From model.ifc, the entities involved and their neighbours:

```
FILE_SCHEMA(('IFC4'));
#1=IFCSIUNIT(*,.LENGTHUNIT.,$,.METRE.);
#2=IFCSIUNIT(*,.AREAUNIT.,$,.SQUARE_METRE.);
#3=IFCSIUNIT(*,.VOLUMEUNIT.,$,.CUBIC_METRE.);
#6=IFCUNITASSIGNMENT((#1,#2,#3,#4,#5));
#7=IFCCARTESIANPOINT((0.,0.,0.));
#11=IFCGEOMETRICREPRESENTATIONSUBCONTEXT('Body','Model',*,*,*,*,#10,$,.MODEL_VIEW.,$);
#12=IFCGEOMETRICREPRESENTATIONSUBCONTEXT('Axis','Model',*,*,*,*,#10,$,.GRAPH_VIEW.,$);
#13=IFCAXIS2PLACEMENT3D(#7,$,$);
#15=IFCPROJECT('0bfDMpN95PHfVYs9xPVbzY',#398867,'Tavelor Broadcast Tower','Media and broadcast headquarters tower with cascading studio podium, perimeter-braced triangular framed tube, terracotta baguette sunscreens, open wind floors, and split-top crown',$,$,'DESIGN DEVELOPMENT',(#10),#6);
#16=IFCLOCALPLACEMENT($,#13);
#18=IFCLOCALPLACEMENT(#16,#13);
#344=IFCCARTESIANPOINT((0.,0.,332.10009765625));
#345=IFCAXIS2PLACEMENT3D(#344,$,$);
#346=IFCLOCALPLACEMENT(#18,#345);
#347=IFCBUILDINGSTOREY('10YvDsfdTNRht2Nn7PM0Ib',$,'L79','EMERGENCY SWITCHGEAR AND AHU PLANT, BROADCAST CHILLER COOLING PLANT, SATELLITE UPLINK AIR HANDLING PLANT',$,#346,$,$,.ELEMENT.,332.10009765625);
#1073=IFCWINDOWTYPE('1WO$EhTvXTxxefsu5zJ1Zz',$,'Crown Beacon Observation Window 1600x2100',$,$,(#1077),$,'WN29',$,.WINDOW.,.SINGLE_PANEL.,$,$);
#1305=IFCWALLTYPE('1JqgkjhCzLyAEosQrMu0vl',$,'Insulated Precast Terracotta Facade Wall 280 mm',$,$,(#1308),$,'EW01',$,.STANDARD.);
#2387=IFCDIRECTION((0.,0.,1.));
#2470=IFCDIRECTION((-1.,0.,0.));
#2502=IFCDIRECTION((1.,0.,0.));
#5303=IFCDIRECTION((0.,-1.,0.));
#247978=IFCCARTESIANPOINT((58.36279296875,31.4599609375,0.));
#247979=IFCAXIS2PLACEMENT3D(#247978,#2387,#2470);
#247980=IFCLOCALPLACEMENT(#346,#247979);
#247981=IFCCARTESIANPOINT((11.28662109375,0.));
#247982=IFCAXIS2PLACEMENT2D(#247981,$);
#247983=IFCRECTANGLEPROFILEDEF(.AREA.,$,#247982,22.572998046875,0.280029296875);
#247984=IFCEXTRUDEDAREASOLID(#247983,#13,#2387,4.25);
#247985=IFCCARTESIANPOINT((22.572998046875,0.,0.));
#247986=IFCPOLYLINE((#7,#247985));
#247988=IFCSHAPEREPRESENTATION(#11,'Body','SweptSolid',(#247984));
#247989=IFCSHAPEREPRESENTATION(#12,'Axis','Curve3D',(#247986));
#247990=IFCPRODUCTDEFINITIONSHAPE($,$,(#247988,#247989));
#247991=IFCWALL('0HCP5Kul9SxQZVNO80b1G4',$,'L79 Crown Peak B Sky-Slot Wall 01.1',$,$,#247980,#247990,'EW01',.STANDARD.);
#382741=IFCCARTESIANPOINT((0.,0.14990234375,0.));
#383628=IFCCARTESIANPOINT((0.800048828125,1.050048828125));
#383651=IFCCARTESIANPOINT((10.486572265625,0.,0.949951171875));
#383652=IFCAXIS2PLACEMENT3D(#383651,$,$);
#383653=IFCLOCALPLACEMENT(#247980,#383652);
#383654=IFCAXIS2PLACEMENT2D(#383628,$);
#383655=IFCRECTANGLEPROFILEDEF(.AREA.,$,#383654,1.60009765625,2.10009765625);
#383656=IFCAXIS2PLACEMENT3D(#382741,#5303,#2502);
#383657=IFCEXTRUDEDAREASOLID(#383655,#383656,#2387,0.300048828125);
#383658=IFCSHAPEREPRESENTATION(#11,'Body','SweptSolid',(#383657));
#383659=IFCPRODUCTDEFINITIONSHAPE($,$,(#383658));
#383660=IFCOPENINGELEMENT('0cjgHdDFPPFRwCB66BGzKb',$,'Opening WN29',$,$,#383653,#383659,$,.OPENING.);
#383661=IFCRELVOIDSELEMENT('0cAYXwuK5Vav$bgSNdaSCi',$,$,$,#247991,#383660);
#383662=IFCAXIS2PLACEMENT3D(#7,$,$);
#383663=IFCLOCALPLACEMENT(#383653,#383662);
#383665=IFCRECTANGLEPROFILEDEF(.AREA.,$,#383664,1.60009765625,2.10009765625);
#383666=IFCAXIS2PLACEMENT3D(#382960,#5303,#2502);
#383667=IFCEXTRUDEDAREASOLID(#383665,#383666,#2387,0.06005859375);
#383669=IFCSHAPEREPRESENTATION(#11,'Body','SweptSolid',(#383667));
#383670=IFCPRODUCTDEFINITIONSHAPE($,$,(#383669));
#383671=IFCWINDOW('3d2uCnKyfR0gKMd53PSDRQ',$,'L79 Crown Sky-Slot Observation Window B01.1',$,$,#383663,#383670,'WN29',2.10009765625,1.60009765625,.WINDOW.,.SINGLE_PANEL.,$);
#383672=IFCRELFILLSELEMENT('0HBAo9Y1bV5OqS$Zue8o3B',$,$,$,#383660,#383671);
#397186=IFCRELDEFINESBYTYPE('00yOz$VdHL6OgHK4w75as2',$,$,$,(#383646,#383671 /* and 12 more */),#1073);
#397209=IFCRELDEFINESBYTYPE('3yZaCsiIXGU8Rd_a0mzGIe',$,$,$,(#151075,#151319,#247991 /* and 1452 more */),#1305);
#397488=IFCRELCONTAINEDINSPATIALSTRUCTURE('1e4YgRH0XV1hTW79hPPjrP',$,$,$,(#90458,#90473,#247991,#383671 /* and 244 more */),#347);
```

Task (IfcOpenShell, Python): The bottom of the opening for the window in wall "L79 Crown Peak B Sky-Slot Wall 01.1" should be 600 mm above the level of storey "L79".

```python
import numpy as np
import ifcopenshell
import ifcopenshell.api.geometry
import ifcopenshell.geom
import ifcopenshell.util.element
import ifcopenshell.util.placement
import ifcopenshell.util.shape
import ifcopenshell.util.unit

model = ifcopenshell.open("model.ifc")
unit_scale = ifcopenshell.util.unit.calculate_unit_scale(model)

window = model.by_guid("3d2uCnKyfR0gKMd53PSDRQ")
opening = window.FillsVoids[0].RelatingOpeningElement
storey = ifcopenshell.util.element.get_container(window, ifc_class="IfcBuildingStorey")
level = ifcopenshell.util.placement.get_local_placement(storey.ObjectPlacement)[2, 3]

# The opening's origin need not be at the sill, so measure its lowest point.
shape = ifcopenshell.geom.create_shape(ifcopenshell.geom.settings(), opening)
bottom = ifcopenshell.util.shape.get_shape_bottom_elevation(shape, shape.geometry) / unit_scale
dz = level + 0.6 - bottom

shift = np.array([0.0, 0.0, dz])
# The window is placed relative to its opening, so it follows when the opening moves.
matrix = ifcopenshell.util.placement.get_local_placement(opening.ObjectPlacement)
matrix[:3, 3] += shift
ifcopenshell.api.geometry.edit_object_placement(
    model, product=opening, matrix=matrix, is_si=False, should_transform_children=True
)

print(f"moved by {dz * unit_scale:+.3f} m")

model.write("model_updated.ifc")
```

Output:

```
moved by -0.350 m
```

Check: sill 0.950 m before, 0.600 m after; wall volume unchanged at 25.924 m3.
